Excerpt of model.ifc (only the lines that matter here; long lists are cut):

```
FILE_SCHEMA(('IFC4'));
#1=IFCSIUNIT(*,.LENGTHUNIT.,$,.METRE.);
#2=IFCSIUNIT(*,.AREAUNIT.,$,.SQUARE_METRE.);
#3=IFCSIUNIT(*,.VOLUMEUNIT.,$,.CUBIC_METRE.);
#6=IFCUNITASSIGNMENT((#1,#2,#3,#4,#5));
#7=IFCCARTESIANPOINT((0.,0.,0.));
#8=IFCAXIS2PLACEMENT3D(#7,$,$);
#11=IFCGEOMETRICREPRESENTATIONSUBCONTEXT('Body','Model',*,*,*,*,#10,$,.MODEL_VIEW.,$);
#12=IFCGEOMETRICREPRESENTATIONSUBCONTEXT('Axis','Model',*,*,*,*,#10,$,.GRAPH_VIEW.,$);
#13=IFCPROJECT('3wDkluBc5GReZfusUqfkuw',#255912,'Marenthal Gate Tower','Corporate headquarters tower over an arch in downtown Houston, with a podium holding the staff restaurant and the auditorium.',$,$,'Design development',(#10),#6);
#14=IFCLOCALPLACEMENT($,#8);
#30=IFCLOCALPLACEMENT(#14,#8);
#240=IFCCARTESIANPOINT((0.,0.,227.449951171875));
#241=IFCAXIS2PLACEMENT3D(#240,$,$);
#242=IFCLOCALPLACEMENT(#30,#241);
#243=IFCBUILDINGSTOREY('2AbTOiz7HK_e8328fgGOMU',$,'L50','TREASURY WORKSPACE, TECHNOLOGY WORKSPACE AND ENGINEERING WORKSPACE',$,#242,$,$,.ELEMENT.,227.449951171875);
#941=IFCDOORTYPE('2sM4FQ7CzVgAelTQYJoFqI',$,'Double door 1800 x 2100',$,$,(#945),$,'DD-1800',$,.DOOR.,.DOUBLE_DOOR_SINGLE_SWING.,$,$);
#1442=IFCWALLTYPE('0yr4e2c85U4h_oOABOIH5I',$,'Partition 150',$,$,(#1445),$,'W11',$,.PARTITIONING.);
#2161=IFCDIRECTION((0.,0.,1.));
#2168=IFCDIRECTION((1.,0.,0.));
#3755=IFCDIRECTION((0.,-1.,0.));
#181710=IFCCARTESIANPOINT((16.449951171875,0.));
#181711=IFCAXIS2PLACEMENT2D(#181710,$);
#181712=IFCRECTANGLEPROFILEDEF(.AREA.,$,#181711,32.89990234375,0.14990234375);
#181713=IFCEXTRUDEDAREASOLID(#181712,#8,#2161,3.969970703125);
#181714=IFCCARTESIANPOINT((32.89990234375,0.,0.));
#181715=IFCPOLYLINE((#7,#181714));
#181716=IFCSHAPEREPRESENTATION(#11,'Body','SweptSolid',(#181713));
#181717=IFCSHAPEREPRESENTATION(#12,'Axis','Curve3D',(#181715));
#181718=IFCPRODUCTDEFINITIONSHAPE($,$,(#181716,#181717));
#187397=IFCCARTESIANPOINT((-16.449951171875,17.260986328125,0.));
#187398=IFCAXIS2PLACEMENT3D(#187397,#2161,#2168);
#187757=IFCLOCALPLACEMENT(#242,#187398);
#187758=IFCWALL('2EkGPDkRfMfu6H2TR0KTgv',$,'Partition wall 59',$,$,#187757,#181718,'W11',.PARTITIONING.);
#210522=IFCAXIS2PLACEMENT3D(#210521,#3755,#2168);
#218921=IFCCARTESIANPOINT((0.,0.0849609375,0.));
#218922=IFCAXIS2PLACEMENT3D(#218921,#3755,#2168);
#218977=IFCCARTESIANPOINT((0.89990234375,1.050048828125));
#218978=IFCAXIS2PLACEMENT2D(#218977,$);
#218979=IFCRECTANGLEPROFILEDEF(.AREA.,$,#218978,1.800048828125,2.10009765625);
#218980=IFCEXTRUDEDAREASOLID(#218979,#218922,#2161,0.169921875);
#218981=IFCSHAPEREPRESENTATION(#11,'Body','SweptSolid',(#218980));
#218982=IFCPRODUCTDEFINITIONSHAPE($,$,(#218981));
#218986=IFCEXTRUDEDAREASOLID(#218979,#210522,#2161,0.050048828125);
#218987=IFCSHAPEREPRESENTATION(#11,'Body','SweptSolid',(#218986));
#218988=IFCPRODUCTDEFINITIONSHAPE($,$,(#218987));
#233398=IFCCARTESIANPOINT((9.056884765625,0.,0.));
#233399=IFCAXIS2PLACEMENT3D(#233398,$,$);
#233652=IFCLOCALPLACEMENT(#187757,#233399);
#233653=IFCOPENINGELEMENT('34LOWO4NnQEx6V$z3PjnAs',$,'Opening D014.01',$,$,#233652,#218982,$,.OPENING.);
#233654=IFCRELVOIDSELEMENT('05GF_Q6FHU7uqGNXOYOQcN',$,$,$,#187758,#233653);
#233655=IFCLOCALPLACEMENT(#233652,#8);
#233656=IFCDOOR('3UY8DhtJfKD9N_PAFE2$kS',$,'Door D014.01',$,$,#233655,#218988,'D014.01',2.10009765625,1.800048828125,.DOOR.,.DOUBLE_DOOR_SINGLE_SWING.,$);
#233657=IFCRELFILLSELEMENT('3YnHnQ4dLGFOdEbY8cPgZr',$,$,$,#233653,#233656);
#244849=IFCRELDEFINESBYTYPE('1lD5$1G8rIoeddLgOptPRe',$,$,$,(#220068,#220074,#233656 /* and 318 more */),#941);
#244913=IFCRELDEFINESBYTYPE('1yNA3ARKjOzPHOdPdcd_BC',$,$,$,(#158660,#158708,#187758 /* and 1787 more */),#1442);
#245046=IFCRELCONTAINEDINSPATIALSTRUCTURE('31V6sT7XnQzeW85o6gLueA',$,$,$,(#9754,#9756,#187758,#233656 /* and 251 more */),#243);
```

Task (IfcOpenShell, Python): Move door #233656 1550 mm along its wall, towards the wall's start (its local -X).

```python
import ifcopenshell
import ifcopenshell.api.geometry
import ifcopenshell.util.placement

model = ifcopenshell.open("model.ifc")

door = model.by_guid("3UY8DhtJfKD9N_PAFE2$kS")
opening = door.FillsVoids[0].RelatingOpeningElement
wall = opening.VoidsElements[0].RelatingBuildingElement

wall_matrix = ifcopenshell.util.placement.get_local_placement(wall.ObjectPlacement)
shift = wall_matrix[:3, 0] * -1.55
before = ifcopenshell.util.placement.get_local_placement(door.ObjectPlacement)[:3, 3].copy()

# The door is placed relative to its opening, so it follows when the opening moves.
matrix = ifcopenshell.util.placement.get_local_placement(opening.ObjectPlacement)
matrix[:3, 3] += shift
ifcopenshell.api.geometry.edit_object_placement(
    model, product=opening, matrix=matrix, is_si=False, should_transform_children=True
)

after = ifcopenshell.util.placement.get_local_placement(door.ObjectPlacement)[:3, 3]
print("door moved by", (after - before).round(3) + 0.0)

model.write("model_v2.ifc")
```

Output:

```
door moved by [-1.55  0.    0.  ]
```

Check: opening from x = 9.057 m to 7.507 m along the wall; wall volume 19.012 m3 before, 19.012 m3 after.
